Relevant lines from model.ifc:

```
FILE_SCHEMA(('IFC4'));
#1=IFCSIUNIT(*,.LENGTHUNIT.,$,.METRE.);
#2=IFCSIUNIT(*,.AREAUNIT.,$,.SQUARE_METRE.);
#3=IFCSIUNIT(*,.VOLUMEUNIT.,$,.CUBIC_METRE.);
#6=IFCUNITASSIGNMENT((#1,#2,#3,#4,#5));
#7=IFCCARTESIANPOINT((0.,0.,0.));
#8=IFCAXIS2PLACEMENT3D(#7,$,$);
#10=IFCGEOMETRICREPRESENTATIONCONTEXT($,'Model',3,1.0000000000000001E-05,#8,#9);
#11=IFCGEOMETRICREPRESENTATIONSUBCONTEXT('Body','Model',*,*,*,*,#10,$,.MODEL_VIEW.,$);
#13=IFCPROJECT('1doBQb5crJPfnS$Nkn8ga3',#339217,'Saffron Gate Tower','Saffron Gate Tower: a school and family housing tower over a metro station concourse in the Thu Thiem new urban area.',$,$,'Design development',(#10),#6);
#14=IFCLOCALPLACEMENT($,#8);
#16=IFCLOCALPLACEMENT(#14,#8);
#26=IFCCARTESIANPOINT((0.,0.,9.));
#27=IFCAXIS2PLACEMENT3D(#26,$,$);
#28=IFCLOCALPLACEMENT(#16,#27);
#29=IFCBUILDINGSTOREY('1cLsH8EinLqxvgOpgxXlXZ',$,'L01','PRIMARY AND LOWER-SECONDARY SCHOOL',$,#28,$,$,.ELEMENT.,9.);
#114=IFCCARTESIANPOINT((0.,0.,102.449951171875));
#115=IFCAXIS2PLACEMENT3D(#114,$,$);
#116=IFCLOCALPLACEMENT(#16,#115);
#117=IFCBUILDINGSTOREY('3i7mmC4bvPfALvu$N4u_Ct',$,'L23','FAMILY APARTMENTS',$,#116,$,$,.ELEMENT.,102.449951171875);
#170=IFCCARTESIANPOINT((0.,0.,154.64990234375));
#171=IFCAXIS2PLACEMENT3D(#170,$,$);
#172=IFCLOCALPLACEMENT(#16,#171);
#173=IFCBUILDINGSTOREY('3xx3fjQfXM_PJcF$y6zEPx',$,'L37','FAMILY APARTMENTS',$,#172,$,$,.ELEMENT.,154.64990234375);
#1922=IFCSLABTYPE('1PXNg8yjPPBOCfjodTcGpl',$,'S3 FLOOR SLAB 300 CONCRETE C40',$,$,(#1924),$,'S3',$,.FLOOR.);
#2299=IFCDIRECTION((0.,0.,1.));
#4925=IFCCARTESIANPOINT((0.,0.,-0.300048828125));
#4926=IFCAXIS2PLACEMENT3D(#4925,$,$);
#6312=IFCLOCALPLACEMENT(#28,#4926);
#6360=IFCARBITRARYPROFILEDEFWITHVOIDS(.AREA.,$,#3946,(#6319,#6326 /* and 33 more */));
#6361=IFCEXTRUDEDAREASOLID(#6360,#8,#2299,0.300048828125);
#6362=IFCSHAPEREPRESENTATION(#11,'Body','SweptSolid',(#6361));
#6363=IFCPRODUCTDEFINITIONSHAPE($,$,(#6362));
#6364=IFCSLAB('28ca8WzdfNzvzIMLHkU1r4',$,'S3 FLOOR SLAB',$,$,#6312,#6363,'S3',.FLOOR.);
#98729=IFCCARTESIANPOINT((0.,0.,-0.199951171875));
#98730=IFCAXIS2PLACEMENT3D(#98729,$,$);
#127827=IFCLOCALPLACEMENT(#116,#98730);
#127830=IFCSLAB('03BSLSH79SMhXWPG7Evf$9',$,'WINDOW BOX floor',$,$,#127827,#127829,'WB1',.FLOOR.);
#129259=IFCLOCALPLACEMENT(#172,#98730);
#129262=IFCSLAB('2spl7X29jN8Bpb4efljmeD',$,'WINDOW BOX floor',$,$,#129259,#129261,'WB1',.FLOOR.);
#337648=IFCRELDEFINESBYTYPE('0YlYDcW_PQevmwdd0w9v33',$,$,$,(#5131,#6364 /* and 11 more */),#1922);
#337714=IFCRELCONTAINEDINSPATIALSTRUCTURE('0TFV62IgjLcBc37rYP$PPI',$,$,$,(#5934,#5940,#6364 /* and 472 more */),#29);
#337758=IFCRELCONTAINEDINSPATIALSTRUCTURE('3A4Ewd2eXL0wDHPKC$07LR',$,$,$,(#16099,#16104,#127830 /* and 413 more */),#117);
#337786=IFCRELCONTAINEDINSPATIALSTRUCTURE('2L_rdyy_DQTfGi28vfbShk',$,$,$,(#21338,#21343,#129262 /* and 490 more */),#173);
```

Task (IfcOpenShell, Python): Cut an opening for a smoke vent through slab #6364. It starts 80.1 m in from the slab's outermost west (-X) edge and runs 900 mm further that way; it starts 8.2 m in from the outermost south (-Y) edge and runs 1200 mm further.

```python
import numpy as np
import ifcopenshell
import ifcopenshell.api.feature
import ifcopenshell.api.geometry
import ifcopenshell.api.root
import ifcopenshell.geom
import ifcopenshell.util.placement
import ifcopenshell.util.representation
import ifcopenshell.util.shape
import ifcopenshell.util.unit

model = ifcopenshell.open("model.ifc")
unit_scale = ifcopenshell.util.unit.calculate_unit_scale(model)
settings = ifcopenshell.geom.settings()


def volume(element):
    """Net volume in cubic metres, openings subtracted."""
    shape = ifcopenshell.geom.create_shape(settings, element)
    return ifcopenshell.util.shape.get_volume(shape.geometry)


slab = model.by_guid("28ca8WzdfNzvzIMLHkU1r4")
before = volume(slab)

# Extent in the slab's own axes, in metres. The edges named are its -X and -Y sides.
slab_shape = ifcopenshell.geom.create_shape(settings, slab)
vertices = ifcopenshell.util.shape.get_vertices(slab_shape.geometry)
x_min, y_min, bottom = vertices.min(axis=0)
top = vertices[:, 2].max()

opening = ifcopenshell.api.root.create_entity(model, ifc_class="IfcOpeningElement", name="Smoke vent opening", predefined_type="OPENING")
context = ifcopenshell.util.representation.get_context(model, "Model", "Body", "MODEL_VIEW")
width, depth = 0.9, 1.2
outline = [(0.0, 0.0), (width, 0.0), (width, depth), (0.0, depth), (0.0, 0.0)]
# Overshoot both faces by 50 mm so the cut is clean.
shape = ifcopenshell.api.geometry.add_slab_representation(
    model, context=context, depth=top - bottom + 0.1, polyline=outline
)
ifcopenshell.api.geometry.assign_representation(model, product=opening, representation=shape)

matrix = ifcopenshell.util.placement.get_local_placement(slab.ObjectPlacement)
matrix[:, 3] = matrix @ np.append(np.array([x_min + 80.1, y_min + 8.2, bottom - 0.05]) / unit_scale, 1.0)
ifcopenshell.api.geometry.edit_object_placement(model, product=opening, matrix=matrix, is_si=False)
ifcopenshell.api.feature.add_feature(model, feature=opening, element=slab)

after = volume(slab)

print(f"slab volume {before:.3f} -> {after:.3f} m3")

model.write("model_v2.ifc")
```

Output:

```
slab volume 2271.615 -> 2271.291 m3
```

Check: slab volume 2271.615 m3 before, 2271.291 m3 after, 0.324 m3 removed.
